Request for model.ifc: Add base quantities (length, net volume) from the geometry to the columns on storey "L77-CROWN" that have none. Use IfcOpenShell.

First a look at what the model holds.

```python
import ifcopenshell
import ifcopenshell.util.element
import ifcopenshell.util.unit

model = ifcopenshell.open("model.ifc")
print(model.schema)
for unit_type in ("LENGTHUNIT", "AREAUNIT", "VOLUMEUNIT"):
    print(unit_type, ifcopenshell.util.unit.calculate_unit_scale(model, unit_type))
storey = next(s for s in model.by_type("IfcBuildingStorey") if s.Name == "L77-CROWN")
columns = [e for e in ifcopenshell.util.element.get_decomposition(storey) if e.is_a("IfcColumn")]
for e in sorted(columns, key=lambda e: e.id()):
    print(e.id(), e.is_a(), e.Name, list(ifcopenshell.util.element.get_psets(e, qtos_only=True)), sep=" | ")
```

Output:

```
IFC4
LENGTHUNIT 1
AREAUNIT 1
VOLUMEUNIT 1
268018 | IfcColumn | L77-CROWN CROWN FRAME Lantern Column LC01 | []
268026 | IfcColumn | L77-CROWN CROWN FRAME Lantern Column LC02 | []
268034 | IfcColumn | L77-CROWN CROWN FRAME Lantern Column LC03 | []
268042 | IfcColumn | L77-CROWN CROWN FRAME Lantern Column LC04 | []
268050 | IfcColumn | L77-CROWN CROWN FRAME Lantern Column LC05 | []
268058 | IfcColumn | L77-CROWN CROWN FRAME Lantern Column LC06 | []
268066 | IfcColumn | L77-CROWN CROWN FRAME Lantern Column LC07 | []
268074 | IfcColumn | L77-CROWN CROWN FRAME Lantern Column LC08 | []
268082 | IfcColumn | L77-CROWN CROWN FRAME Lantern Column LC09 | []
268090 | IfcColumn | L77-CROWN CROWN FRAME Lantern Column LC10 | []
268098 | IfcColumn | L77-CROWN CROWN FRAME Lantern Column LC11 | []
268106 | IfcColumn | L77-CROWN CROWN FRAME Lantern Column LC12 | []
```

```python
import ifcopenshell
import ifcopenshell.api.pset
import ifcopenshell.geom
import ifcopenshell.util.element
import ifcopenshell.util.shape
import ifcopenshell.util.unit

model = ifcopenshell.open("model.ifc")
unit_scale = ifcopenshell.util.unit.calculate_unit_scale(model)
volume_scale = ifcopenshell.util.unit.calculate_unit_scale(model, "VOLUMEUNIT")
settings = ifcopenshell.geom.settings()

storey = next(s for s in model.by_type("IfcBuildingStorey") if s.Name == "L77-CROWN")
columns = [e for e in ifcopenshell.util.element.get_decomposition(storey) if e.is_a("IfcColumn")]

for e in sorted(columns, key=lambda e: e.id()):
    if ifcopenshell.util.element.get_psets(e, qtos_only=True, should_inherit=False):
        continue
    # Geometry comes back in metres, in the element's own axes.
    shape = ifcopenshell.geom.create_shape(settings, e)
    values = {
        "Length": ifcopenshell.util.shape.get_z(shape.geometry) / unit_scale,
        "NetVolume": ifcopenshell.util.shape.get_volume(shape.geometry) / volume_scale,
    }
    qto = ifcopenshell.api.pset.add_qto(model, product=e, name="Qto_ColumnBaseQuantities")
    ifcopenshell.api.pset.edit_qto(model, qto=qto, properties=values)
    print(e.id(), {k: round(v, 3) for k, v in values.items()})

model.write("model_edited.ifc")
```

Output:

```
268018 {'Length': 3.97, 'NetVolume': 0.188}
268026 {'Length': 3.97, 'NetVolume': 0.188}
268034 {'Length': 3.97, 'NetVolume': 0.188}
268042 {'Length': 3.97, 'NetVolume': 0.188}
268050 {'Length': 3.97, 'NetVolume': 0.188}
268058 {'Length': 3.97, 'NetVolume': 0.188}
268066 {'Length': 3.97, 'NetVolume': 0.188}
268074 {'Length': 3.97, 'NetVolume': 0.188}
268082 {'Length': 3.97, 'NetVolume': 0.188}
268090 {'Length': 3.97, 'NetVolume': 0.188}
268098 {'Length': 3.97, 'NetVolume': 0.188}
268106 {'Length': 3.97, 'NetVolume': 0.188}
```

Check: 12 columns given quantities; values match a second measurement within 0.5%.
